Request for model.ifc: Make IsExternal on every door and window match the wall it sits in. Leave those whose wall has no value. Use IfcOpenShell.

First a look at what the model holds.

```python
import ifcopenshell
import ifcopenshell.util.element

model = ifcopenshell.open("model.ifc")
print(model.schema)
seen = {}
for e in model.by_type("IfcDoor") + model.by_type("IfcWindow"):
    if not e.FillsVoids:
        continue
    host = e.FillsVoids[0].RelatingOpeningElement.VoidsElements[0].RelatingBuildingElement
    own = ifcopenshell.util.element.get_pset(e, f"Pset_{e.is_a()[3:].removesuffix('StandardCase')}Common", "IsExternal")
    wall = ifcopenshell.util.element.get_pset(host, "Pset_WallCommon", "IsExternal")
    seen[e.is_a(), own, wall] = seen.get((e.is_a(), own, wall), 0) + 1
for (cls, own, wall), count in sorted(seen.items(), key=str):
    print(count, cls, "IsExternal:", own, "| host wall:", wall)
```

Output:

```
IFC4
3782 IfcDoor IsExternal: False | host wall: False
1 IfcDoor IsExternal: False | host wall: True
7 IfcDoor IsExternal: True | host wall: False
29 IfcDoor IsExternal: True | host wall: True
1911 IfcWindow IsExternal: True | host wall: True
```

```python
import ifcopenshell
import ifcopenshell.api.pset
import ifcopenshell.util.element

model = ifcopenshell.open("model.ifc")

count = 0
for ifc_class, pset_name in (("IfcDoor", "Pset_DoorCommon"), ("IfcWindow", "Pset_WindowCommon")):
    for e in model.by_type(ifc_class):
        if not e.FillsVoids:
            continue
        host = e.FillsVoids[0].RelatingOpeningElement.VoidsElements[0].RelatingBuildingElement
        external = ifcopenshell.util.element.get_pset(host, "Pset_WallCommon", "IsExternal")
        if external is None or ifcopenshell.util.element.get_pset(e, pset_name, "IsExternal") == external:
            continue
        pset = ifcopenshell.api.pset.add_pset(model, product=e, name=pset_name)
        ifcopenshell.api.pset.edit_pset(model, pset=pset, properties={"IsExternal": external})
        count += 1

print(count, "updated")

model.write("model_updated.ifc")
```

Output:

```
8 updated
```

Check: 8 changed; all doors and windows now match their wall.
